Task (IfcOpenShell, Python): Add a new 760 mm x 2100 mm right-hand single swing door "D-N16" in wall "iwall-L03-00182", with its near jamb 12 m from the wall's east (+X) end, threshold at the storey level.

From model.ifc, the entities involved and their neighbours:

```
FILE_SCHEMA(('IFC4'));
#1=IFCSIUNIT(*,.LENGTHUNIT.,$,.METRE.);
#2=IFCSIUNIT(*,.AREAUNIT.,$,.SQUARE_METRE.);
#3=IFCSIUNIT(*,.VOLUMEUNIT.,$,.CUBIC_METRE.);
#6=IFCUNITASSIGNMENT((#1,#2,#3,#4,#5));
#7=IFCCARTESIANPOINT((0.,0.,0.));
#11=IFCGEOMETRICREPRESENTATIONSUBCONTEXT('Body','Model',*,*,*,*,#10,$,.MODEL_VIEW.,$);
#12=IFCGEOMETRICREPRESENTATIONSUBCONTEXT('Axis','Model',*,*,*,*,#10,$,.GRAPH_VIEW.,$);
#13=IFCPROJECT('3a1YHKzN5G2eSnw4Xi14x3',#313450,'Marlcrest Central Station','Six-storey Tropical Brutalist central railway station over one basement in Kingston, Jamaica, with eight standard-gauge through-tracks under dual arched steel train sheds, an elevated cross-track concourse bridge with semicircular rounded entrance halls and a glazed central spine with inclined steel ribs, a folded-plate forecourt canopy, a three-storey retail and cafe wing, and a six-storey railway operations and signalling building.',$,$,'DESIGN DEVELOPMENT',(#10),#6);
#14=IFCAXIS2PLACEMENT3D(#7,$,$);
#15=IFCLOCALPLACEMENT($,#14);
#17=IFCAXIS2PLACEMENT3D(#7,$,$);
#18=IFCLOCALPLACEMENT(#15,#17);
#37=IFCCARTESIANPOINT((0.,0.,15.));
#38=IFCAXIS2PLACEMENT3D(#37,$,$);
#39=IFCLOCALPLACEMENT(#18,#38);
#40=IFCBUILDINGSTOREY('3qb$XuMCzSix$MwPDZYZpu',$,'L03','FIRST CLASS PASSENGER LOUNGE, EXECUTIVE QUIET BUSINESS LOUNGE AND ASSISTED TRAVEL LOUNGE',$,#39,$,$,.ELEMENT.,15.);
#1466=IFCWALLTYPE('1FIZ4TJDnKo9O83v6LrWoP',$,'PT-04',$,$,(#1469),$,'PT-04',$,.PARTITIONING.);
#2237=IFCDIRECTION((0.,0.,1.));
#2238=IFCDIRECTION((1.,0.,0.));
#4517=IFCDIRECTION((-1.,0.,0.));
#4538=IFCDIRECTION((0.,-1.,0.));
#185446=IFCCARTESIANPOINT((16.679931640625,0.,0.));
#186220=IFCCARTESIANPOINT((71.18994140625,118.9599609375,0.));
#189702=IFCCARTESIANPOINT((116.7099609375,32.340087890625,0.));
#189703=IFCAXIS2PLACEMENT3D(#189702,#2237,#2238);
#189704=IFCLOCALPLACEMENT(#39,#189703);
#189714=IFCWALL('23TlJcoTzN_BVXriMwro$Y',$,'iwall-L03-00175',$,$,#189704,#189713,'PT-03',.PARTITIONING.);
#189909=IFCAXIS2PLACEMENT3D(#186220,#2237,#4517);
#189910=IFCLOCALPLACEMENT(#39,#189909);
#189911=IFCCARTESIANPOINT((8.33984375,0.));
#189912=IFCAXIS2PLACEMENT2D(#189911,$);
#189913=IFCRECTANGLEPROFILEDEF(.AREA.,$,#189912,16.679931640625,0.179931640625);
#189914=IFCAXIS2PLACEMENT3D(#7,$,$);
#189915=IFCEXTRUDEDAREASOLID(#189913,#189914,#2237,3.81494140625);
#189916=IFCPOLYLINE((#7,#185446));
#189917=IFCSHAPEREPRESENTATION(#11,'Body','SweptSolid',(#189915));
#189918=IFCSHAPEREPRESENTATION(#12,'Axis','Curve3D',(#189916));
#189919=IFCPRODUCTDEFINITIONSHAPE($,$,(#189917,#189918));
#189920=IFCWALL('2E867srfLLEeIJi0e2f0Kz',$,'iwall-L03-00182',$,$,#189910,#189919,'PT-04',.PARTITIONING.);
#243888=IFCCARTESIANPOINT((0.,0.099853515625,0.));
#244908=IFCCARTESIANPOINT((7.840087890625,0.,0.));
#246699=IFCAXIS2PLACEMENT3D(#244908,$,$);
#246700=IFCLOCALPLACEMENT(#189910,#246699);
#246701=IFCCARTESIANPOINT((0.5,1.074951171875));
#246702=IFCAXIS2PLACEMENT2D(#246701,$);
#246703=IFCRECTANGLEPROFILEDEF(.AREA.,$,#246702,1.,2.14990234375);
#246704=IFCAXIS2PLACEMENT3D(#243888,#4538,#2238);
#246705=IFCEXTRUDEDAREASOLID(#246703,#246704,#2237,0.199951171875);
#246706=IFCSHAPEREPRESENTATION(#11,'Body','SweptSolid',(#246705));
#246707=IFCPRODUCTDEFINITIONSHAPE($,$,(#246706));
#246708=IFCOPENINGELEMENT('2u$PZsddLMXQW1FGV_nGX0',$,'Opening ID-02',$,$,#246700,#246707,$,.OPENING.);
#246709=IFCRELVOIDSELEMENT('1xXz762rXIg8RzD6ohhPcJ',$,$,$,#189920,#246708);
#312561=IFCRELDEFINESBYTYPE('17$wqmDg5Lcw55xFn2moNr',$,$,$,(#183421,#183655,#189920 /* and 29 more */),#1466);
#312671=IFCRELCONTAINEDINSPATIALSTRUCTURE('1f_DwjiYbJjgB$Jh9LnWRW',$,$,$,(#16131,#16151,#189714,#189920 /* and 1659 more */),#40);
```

```python
import numpy as np
import ifcopenshell
import ifcopenshell.api.feature
import ifcopenshell.api.geometry
import ifcopenshell.api.root
import ifcopenshell.api.spatial
import ifcopenshell.geom
import ifcopenshell.util.element
import ifcopenshell.util.placement
import ifcopenshell.util.representation
import ifcopenshell.util.shape
import ifcopenshell.util.unit

model = ifcopenshell.open("model.ifc")
unit_scale = ifcopenshell.util.unit.calculate_unit_scale(model)
settings = ifcopenshell.geom.settings()


def volume(element):
    """Net volume in cubic metres, openings subtracted."""
    shape = ifcopenshell.geom.create_shape(settings, element)
    return ifcopenshell.util.shape.get_volume(shape.geometry)


wall = model.by_guid("2E867srfLLEeIJi0e2f0Kz")
storey = ifcopenshell.util.element.get_container(wall, ifc_class="IfcBuildingStorey")
context = ifcopenshell.util.representation.get_context(model, "Model", "Body", "MODEL_VIEW")
before = volume(wall)

width, height, from_end, sill = 0.76, 2.1, 12, 0.0  # metres

# The wall runs along its own X axis, and the end named is its -X end.
wall_shape = ifcopenshell.geom.create_shape(settings, wall)
x, y, z = ifcopenshell.util.shape.get_vertices(wall_shape.geometry).T
start = x.min() + from_end
face, thickness = float(y.min()), float(y.max() - y.min())
wall_matrix = ifcopenshell.util.placement.get_local_placement(wall.ObjectPlacement)
level = ifcopenshell.util.placement.get_local_placement(storey.ObjectPlacement)[2, 3]


def in_wall(x, y):
    """Placement at x, y metres in the wall's axes, at sill height."""
    matrix = wall_matrix.copy()
    matrix[:, 3] = wall_matrix @ np.array([x / unit_scale, y / unit_scale, 0.0, 1.0])
    matrix[2, 3] = level + sill / unit_scale
    return matrix


# Opening: a box that overshoots both wall faces by 50 mm.
opening = ifcopenshell.api.root.create_entity(model, ifc_class="IfcOpeningElement", predefined_type="OPENING")
box = ifcopenshell.api.geometry.add_wall_representation(
    model, context=context, length=width, height=height, thickness=thickness + 0.1
)
ifcopenshell.api.geometry.assign_representation(model, product=opening, representation=box)
ifcopenshell.api.geometry.edit_object_placement(model, product=opening, matrix=in_wall(start, face - 0.05), is_si=False)
ifcopenshell.api.feature.add_feature(model, feature=opening, element=wall)

door = ifcopenshell.api.root.create_entity(model, ifc_class="IfcDoor", name="D-N16", predefined_type="DOOR")
door.OverallWidth, door.OverallHeight = width / unit_scale, height / unit_scale
door.OperationType = "SINGLE_SWING_RIGHT"
body = ifcopenshell.api.geometry.add_door_representation(
    model,
    context=context,
    overall_width=door.OverallWidth,
    overall_height=door.OverallHeight,
    operation_type="SINGLE_SWING_RIGHT",
    lining_properties={"LiningDepth": thickness / unit_scale, "ThresholdDepth": thickness / unit_scale},
)
ifcopenshell.api.geometry.assign_representation(model, product=door, representation=body)
ifcopenshell.api.spatial.assign_container(model, products=[door], relating_structure=storey)
ifcopenshell.api.feature.add_filling(model, opening=opening, element=door)

# The lining spans the wall, so the door starts at the wall face.
ifcopenshell.api.geometry.edit_object_placement(model, product=door, matrix=in_wall(start, face), is_si=False)

after = volume(wall)

print(f"wall volume {before:.3f} -> {after:.3f} m3")

model.write("model_updated.ifc")
```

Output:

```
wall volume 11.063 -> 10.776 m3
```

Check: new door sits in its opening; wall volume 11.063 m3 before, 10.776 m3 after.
